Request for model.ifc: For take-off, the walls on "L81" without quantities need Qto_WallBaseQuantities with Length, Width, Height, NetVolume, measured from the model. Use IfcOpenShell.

First a look at what the model holds.

```python
import ifcopenshell
import ifcopenshell.util.element
import ifcopenshell.util.unit

model = ifcopenshell.open("model.ifc")
print(model.schema)
for unit_type in ("LENGTHUNIT", "AREAUNIT", "VOLUMEUNIT"):
    print(unit_type, ifcopenshell.util.unit.calculate_unit_scale(model, unit_type))
storey = next(s for s in model.by_type("IfcBuildingStorey") if s.Name == "L81")
walls = [e for e in ifcopenshell.util.element.get_decomposition(storey) if e.is_a("IfcWall")]
for e in sorted(walls, key=lambda e: e.id()):
    print(e.id(), e.is_a(), e.Name, list(ifcopenshell.util.element.get_psets(e, qtos_only=True)), sep=" | ")
```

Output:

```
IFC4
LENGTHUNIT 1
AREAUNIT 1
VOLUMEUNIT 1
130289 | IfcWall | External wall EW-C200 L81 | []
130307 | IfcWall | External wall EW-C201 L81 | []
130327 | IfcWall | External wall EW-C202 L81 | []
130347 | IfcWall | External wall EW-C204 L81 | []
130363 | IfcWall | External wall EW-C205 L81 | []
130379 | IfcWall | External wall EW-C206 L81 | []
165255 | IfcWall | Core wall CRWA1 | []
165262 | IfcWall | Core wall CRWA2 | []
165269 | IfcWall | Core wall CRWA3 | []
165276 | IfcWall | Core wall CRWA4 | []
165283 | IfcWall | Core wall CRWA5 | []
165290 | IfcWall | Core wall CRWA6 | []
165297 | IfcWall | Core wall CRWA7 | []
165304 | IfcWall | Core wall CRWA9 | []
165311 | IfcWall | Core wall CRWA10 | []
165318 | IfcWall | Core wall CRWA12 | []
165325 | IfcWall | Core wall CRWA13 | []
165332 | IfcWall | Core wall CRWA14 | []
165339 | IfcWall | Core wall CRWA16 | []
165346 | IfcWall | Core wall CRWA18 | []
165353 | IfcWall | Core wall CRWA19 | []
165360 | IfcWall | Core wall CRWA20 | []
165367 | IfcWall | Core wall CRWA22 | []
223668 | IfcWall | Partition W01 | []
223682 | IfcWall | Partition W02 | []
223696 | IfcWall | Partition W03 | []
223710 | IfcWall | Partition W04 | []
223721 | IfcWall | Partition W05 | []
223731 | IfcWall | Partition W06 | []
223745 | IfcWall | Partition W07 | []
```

```python
import ifcopenshell
import ifcopenshell.api.pset
import ifcopenshell.geom
import ifcopenshell.util.element
import ifcopenshell.util.shape
import ifcopenshell.util.unit

model = ifcopenshell.open("model.ifc")
unit_scale = ifcopenshell.util.unit.calculate_unit_scale(model)
volume_scale = ifcopenshell.util.unit.calculate_unit_scale(model, "VOLUMEUNIT")
settings = ifcopenshell.geom.settings()

storey = next(s for s in model.by_type("IfcBuildingStorey") if s.Name == "L81")
walls = [e for e in ifcopenshell.util.element.get_decomposition(storey) if e.is_a("IfcWall")]

for e in sorted(walls, key=lambda e: e.id()):
    if ifcopenshell.util.element.get_psets(e, qtos_only=True, should_inherit=False):
        continue
    # Geometry comes back in metres, in the element's own axes.
    shape = ifcopenshell.geom.create_shape(settings, e)
    values = {
        "Length": ifcopenshell.util.shape.get_x(shape.geometry) / unit_scale,
        "Width": ifcopenshell.util.shape.get_y(shape.geometry) / unit_scale,
        "Height": ifcopenshell.util.shape.get_z(shape.geometry) / unit_scale,
        "NetVolume": ifcopenshell.util.shape.get_volume(shape.geometry) / volume_scale,
    }
    qto = ifcopenshell.api.pset.add_qto(model, product=e, name="Qto_WallBaseQuantities")
    ifcopenshell.api.pset.edit_qto(model, qto=qto, properties=values)
    print(e.id(), {k: round(v, 3) for k, v in values.items()})

model.write("model_edited.ifc")
```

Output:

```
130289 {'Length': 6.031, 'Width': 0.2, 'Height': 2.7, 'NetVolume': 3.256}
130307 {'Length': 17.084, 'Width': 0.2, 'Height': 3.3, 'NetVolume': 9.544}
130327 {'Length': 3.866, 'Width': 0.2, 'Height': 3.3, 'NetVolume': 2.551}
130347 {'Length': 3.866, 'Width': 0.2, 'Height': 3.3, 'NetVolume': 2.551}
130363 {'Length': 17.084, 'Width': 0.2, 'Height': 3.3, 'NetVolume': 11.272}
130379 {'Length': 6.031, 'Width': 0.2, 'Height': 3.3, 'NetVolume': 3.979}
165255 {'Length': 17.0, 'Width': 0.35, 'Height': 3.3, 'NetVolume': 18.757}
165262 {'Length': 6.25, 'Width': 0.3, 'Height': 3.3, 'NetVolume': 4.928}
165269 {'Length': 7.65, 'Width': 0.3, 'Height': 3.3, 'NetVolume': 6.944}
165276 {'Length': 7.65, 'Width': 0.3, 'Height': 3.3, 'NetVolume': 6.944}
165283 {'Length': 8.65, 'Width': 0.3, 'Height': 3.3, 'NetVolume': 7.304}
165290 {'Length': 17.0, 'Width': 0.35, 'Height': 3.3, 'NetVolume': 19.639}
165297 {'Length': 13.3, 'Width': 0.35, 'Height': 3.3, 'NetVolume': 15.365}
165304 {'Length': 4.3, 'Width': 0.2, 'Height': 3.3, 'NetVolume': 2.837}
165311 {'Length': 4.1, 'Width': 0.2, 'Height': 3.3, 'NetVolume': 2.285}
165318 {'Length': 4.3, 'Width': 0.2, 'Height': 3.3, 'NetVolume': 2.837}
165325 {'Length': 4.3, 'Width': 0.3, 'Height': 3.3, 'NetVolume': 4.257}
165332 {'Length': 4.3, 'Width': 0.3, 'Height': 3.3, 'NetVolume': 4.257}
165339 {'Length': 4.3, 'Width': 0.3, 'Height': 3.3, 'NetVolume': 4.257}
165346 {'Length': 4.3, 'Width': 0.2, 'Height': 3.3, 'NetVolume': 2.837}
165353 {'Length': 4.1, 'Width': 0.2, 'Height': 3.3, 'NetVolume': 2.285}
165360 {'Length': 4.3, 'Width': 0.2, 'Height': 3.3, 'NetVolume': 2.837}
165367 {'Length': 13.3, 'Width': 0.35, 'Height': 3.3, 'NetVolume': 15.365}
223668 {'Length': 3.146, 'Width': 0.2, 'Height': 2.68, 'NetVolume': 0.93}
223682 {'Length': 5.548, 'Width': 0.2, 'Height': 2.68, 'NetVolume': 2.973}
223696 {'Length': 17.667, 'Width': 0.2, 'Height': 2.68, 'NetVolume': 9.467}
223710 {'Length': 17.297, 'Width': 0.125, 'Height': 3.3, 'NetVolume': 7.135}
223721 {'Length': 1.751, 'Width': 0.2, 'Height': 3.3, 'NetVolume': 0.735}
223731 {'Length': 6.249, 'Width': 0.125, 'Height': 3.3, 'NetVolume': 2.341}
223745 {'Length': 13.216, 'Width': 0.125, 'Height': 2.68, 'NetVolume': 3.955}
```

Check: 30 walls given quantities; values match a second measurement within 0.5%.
